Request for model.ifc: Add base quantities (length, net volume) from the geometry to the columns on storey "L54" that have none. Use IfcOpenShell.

First a look at what the model holds.

```python
import ifcopenshell
import ifcopenshell.util.element
import ifcopenshell.util.unit

model = ifcopenshell.open("model.ifc")
print(model.schema)
for unit_type in ("LENGTHUNIT", "AREAUNIT", "VOLUMEUNIT"):
    print(unit_type, ifcopenshell.util.unit.calculate_unit_scale(model, unit_type))
storey = next(s for s in model.by_type("IfcBuildingStorey") if s.Name == "L54")
columns = [e for e in ifcopenshell.util.element.get_decomposition(storey) if e.is_a("IfcColumn")]
for e in sorted(columns, key=lambda e: e.id()):
    print(e.id(), e.is_a(), e.Name, list(ifcopenshell.util.element.get_psets(e, qtos_only=True)), sep=" | ")
```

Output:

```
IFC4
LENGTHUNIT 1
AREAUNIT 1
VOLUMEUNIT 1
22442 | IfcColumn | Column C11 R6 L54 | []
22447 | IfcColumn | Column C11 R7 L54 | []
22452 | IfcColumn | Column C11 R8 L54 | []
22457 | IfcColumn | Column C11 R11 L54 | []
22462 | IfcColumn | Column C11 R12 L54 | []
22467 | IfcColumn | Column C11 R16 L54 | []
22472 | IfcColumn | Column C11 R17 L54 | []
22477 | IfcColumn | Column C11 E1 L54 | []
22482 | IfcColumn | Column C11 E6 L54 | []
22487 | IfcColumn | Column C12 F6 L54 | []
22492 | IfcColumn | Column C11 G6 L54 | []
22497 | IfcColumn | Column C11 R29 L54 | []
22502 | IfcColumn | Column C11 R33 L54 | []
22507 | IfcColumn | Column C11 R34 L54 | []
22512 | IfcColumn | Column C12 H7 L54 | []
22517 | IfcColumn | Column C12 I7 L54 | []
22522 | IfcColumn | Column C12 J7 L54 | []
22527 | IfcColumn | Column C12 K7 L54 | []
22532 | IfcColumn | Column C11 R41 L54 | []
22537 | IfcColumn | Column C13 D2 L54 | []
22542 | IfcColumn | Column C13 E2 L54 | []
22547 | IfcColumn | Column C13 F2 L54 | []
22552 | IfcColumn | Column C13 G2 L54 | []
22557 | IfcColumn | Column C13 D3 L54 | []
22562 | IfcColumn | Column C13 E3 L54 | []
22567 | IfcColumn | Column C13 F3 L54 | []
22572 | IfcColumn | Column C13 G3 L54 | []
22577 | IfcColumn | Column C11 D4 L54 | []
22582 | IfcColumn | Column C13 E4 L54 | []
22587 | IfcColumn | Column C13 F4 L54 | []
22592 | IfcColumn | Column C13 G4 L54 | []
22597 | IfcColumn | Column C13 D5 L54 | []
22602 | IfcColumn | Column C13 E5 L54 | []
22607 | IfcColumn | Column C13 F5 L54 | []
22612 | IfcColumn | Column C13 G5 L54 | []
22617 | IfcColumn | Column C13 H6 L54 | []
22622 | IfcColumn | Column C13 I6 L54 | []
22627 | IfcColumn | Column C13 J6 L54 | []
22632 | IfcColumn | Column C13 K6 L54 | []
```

```python
import ifcopenshell
import ifcopenshell.api.pset
import ifcopenshell.geom
import ifcopenshell.util.element
import ifcopenshell.util.shape
import ifcopenshell.util.unit

model = ifcopenshell.open("model.ifc")
unit_scale = ifcopenshell.util.unit.calculate_unit_scale(model)
volume_scale = ifcopenshell.util.unit.calculate_unit_scale(model, "VOLUMEUNIT")
settings = ifcopenshell.geom.settings()

storey = next(s for s in model.by_type("IfcBuildingStorey") if s.Name == "L54")
columns = [e for e in ifcopenshell.util.element.get_decomposition(storey) if e.is_a("IfcColumn")]

for e in sorted(columns, key=lambda e: e.id()):
    if ifcopenshell.util.element.get_psets(e, qtos_only=True, should_inherit=False):
        continue
    # Geometry comes back in metres, in the element's own axes.
    shape = ifcopenshell.geom.create_shape(settings, e)
    values = {
        "Length": ifcopenshell.util.shape.get_z(shape.geometry) / unit_scale,
        "NetVolume": ifcopenshell.util.shape.get_volume(shape.geometry) / volume_scale,
    }
    qto = ifcopenshell.api.pset.add_qto(model, product=e, name="Qto_ColumnBaseQuantities")
    ifcopenshell.api.pset.edit_qto(model, qto=qto, properties=values)
    print(e.id(), {k: round(v, 3) for k, v in values.items()})

model.write("model_edited.ifc")
```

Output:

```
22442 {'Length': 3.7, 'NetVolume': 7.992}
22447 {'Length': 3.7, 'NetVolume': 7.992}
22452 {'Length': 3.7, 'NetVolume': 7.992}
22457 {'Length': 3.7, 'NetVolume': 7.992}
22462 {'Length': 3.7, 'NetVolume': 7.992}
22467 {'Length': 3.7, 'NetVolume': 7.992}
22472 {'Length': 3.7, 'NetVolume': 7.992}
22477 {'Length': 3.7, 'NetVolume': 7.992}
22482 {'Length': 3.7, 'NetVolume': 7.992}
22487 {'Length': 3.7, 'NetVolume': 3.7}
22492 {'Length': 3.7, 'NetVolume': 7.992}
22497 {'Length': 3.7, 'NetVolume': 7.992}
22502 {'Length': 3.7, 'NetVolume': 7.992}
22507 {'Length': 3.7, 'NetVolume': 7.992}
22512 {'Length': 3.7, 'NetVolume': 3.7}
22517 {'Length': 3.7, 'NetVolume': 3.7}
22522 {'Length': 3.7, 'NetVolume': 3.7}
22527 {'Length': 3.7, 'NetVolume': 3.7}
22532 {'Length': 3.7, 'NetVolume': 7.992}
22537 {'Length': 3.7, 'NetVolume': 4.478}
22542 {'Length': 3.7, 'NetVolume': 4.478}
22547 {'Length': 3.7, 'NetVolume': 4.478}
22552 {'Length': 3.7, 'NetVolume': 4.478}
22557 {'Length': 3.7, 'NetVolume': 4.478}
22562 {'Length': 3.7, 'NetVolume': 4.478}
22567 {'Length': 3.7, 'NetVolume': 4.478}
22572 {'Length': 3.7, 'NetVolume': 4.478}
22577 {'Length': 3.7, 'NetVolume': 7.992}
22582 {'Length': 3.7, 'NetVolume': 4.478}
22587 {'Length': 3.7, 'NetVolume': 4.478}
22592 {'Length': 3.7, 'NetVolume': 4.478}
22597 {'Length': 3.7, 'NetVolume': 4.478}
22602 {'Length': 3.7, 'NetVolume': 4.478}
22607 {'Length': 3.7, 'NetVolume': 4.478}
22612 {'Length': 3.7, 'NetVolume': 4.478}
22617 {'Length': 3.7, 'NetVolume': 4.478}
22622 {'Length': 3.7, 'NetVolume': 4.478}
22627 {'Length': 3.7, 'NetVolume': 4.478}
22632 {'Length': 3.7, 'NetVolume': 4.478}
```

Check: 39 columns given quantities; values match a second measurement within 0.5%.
